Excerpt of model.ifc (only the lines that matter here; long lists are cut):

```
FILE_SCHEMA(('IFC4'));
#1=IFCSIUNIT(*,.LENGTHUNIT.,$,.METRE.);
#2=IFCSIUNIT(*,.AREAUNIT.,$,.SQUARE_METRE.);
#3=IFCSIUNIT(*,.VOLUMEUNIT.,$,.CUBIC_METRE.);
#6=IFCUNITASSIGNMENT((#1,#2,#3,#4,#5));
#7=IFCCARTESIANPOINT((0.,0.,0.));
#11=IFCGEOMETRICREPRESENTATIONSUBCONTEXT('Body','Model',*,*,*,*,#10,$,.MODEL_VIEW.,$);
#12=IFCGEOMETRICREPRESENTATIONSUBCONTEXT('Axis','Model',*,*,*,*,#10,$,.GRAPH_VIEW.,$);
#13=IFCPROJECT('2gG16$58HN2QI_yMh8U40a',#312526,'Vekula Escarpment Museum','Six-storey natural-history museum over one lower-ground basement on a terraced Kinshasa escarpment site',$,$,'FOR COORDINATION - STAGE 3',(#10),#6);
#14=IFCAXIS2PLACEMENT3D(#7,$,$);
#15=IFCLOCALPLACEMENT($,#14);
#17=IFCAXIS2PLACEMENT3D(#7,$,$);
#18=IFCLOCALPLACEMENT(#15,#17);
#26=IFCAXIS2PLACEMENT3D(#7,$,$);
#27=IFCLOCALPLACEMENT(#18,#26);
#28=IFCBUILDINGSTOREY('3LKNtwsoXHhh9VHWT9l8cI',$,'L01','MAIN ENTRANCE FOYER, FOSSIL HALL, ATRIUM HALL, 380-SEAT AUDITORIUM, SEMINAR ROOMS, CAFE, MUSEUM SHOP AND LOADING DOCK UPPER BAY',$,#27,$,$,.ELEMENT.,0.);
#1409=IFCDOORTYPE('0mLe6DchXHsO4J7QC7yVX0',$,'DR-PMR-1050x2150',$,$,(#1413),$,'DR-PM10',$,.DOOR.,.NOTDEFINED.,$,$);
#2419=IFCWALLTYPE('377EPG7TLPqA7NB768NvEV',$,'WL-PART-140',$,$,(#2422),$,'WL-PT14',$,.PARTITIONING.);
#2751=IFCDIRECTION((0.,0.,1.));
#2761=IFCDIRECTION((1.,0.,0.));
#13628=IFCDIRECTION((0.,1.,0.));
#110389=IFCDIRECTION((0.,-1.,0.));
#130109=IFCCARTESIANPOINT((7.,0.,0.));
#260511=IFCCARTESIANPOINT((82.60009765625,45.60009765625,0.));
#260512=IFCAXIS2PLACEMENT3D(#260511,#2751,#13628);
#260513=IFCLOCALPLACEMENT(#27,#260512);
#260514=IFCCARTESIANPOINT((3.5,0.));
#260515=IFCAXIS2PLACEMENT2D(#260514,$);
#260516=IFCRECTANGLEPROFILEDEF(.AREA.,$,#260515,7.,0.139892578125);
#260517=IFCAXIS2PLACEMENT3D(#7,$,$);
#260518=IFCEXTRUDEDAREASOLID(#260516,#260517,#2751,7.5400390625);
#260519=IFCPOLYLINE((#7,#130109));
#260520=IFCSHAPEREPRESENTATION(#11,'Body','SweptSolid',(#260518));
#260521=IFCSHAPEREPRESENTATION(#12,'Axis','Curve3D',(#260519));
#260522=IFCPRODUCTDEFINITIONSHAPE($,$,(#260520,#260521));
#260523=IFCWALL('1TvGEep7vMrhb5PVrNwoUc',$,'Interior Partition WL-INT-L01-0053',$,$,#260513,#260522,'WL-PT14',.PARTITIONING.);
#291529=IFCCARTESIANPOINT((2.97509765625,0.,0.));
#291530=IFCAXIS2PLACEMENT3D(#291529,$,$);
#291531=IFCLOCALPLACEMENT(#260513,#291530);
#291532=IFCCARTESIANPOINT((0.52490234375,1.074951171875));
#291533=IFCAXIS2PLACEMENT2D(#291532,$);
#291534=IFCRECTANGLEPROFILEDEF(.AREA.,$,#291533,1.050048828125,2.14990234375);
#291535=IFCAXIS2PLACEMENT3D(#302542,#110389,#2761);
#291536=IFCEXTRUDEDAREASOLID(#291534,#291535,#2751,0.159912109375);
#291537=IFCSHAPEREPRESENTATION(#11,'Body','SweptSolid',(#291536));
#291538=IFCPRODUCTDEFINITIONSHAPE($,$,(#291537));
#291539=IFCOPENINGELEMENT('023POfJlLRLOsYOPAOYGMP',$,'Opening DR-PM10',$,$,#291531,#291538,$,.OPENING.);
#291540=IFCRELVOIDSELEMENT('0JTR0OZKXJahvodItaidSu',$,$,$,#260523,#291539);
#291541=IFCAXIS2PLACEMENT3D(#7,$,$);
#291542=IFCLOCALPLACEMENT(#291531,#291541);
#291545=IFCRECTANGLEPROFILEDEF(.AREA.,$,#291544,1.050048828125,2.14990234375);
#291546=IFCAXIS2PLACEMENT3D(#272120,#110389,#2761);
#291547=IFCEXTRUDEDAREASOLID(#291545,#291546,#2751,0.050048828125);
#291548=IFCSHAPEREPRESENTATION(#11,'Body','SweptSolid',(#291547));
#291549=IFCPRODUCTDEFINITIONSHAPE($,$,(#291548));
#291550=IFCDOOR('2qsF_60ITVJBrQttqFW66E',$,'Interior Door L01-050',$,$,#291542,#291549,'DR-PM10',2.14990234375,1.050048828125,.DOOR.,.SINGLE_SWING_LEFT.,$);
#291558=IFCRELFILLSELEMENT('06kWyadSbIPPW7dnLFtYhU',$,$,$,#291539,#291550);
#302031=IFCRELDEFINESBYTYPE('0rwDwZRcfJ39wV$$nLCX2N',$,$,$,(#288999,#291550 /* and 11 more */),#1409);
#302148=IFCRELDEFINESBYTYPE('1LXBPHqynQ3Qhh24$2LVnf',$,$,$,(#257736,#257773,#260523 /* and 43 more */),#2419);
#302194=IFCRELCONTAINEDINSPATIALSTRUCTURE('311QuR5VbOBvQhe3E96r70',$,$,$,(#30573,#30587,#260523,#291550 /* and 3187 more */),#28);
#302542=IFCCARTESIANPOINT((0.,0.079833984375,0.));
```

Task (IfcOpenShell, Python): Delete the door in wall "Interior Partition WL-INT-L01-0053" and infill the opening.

```python
import ifcopenshell
import ifcopenshell.api.feature
import ifcopenshell.api.root
import ifcopenshell.geom
import ifcopenshell.util.shape

model = ifcopenshell.open("model.ifc")
settings = ifcopenshell.geom.settings()


def volume(element):
    """Net volume in cubic metres, openings subtracted."""
    shape = ifcopenshell.geom.create_shape(settings, element)
    return ifcopenshell.util.shape.get_volume(shape.geometry)


door = model.by_id(291550)
opening = door.FillsVoids[0].RelatingOpeningElement
wall = opening.VoidsElements[0].RelatingBuildingElement
before = volume(wall)

ifcopenshell.api.root.remove_product(model, product=door)
ifcopenshell.api.feature.remove_feature(model, feature=opening)

after = volume(wall)

print(f"wall volume {before:.3f} -> {after:.3f} m3")

model.write("model_updated.ifc")
```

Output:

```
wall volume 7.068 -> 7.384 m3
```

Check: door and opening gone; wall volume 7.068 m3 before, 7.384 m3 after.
